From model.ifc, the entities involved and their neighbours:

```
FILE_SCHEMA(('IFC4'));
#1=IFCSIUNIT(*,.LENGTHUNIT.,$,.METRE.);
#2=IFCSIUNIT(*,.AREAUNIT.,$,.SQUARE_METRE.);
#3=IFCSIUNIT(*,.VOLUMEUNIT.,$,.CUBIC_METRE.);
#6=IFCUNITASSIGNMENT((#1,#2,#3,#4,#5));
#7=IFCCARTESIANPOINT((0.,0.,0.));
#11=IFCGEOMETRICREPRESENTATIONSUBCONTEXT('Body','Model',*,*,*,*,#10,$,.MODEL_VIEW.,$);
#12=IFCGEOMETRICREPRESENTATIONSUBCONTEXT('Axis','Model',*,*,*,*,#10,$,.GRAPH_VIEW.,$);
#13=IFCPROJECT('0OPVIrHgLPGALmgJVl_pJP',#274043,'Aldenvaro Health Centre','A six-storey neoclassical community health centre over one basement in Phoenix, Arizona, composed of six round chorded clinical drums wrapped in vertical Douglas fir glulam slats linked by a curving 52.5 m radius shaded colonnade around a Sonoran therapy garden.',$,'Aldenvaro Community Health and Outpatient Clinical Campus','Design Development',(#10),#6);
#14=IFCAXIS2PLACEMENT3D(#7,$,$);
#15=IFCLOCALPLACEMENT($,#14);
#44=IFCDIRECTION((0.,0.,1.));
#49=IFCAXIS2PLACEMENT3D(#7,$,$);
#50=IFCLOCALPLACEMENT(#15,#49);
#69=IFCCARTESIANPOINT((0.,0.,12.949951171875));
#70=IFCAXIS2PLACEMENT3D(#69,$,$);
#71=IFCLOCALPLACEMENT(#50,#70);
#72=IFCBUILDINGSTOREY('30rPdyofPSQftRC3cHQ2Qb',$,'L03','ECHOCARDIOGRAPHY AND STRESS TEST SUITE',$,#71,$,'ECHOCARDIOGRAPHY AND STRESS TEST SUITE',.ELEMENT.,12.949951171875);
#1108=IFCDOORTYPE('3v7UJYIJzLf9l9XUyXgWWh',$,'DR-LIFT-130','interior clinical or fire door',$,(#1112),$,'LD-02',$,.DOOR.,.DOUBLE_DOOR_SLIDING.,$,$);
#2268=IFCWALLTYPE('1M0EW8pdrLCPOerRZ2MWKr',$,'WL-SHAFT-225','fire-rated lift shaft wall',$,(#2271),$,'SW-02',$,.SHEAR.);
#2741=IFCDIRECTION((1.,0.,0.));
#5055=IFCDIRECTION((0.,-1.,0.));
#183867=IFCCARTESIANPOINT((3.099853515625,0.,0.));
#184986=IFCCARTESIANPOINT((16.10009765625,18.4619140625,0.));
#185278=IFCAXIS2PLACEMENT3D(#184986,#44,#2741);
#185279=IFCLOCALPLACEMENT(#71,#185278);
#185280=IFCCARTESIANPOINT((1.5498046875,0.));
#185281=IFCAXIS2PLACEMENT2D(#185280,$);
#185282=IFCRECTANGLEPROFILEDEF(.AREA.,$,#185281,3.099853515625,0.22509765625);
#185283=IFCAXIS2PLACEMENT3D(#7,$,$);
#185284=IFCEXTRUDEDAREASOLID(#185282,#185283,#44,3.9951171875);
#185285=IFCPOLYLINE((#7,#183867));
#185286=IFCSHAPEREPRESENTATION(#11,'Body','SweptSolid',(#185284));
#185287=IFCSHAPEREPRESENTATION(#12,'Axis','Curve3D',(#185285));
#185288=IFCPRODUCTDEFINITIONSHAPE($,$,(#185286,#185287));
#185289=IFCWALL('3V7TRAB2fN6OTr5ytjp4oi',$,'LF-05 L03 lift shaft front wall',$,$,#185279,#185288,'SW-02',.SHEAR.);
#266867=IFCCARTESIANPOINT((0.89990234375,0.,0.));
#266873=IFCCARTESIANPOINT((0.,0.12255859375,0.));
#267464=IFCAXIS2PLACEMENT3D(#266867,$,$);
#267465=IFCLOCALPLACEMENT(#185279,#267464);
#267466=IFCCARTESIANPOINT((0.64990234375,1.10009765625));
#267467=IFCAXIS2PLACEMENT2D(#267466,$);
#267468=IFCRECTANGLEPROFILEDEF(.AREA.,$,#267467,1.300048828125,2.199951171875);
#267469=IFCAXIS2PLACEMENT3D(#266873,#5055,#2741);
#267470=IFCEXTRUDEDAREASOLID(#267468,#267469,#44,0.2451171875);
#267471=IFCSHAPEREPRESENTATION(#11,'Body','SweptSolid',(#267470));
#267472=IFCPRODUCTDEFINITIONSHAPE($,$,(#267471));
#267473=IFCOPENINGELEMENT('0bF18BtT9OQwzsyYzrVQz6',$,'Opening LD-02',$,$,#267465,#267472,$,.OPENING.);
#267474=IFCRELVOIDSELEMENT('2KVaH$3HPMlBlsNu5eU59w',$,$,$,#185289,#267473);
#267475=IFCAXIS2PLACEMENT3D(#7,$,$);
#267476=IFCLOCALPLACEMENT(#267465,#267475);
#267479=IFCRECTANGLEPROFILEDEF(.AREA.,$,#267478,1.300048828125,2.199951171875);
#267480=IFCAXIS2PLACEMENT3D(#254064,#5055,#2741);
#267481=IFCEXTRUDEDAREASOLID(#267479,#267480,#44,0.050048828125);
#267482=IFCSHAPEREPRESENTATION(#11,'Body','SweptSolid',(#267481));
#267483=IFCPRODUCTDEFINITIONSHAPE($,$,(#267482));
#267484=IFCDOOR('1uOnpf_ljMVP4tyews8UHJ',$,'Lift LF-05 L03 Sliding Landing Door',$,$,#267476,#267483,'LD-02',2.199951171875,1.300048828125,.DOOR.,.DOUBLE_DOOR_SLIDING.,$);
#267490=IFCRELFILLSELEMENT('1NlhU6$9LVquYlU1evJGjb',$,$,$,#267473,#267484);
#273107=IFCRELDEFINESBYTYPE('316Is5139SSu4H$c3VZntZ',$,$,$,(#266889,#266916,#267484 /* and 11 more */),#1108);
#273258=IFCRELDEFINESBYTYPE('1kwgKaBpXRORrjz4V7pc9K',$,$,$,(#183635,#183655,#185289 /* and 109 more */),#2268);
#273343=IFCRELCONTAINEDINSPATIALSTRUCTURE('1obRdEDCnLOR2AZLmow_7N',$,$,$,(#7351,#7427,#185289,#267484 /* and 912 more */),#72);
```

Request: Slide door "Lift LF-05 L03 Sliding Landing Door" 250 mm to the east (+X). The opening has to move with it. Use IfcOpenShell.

```python
import ifcopenshell
import ifcopenshell.api.geometry
import ifcopenshell.util.placement

model = ifcopenshell.open("model.ifc")

door = model.by_guid("1uOnpf_ljMVP4tyews8UHJ")
opening = door.FillsVoids[0].RelatingOpeningElement
wall = opening.VoidsElements[0].RelatingBuildingElement

wall_matrix = ifcopenshell.util.placement.get_local_placement(wall.ObjectPlacement)
shift = wall_matrix[:3, 0] * 0.25
before = ifcopenshell.util.placement.get_local_placement(door.ObjectPlacement)[:3, 3].copy()

# The door is placed relative to its opening, so it follows when the opening moves.
matrix = ifcopenshell.util.placement.get_local_placement(opening.ObjectPlacement)
matrix[:3, 3] += shift
ifcopenshell.api.geometry.edit_object_placement(
    model, product=opening, matrix=matrix, is_si=False, should_transform_children=True
)

after = ifcopenshell.util.placement.get_local_placement(door.ObjectPlacement)[:3, 3]
print("door moved by", (after - before).round(3) + 0.0)

model.write("model_rev.ifc")
```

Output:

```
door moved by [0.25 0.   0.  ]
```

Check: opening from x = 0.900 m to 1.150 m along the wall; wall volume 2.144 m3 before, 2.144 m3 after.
